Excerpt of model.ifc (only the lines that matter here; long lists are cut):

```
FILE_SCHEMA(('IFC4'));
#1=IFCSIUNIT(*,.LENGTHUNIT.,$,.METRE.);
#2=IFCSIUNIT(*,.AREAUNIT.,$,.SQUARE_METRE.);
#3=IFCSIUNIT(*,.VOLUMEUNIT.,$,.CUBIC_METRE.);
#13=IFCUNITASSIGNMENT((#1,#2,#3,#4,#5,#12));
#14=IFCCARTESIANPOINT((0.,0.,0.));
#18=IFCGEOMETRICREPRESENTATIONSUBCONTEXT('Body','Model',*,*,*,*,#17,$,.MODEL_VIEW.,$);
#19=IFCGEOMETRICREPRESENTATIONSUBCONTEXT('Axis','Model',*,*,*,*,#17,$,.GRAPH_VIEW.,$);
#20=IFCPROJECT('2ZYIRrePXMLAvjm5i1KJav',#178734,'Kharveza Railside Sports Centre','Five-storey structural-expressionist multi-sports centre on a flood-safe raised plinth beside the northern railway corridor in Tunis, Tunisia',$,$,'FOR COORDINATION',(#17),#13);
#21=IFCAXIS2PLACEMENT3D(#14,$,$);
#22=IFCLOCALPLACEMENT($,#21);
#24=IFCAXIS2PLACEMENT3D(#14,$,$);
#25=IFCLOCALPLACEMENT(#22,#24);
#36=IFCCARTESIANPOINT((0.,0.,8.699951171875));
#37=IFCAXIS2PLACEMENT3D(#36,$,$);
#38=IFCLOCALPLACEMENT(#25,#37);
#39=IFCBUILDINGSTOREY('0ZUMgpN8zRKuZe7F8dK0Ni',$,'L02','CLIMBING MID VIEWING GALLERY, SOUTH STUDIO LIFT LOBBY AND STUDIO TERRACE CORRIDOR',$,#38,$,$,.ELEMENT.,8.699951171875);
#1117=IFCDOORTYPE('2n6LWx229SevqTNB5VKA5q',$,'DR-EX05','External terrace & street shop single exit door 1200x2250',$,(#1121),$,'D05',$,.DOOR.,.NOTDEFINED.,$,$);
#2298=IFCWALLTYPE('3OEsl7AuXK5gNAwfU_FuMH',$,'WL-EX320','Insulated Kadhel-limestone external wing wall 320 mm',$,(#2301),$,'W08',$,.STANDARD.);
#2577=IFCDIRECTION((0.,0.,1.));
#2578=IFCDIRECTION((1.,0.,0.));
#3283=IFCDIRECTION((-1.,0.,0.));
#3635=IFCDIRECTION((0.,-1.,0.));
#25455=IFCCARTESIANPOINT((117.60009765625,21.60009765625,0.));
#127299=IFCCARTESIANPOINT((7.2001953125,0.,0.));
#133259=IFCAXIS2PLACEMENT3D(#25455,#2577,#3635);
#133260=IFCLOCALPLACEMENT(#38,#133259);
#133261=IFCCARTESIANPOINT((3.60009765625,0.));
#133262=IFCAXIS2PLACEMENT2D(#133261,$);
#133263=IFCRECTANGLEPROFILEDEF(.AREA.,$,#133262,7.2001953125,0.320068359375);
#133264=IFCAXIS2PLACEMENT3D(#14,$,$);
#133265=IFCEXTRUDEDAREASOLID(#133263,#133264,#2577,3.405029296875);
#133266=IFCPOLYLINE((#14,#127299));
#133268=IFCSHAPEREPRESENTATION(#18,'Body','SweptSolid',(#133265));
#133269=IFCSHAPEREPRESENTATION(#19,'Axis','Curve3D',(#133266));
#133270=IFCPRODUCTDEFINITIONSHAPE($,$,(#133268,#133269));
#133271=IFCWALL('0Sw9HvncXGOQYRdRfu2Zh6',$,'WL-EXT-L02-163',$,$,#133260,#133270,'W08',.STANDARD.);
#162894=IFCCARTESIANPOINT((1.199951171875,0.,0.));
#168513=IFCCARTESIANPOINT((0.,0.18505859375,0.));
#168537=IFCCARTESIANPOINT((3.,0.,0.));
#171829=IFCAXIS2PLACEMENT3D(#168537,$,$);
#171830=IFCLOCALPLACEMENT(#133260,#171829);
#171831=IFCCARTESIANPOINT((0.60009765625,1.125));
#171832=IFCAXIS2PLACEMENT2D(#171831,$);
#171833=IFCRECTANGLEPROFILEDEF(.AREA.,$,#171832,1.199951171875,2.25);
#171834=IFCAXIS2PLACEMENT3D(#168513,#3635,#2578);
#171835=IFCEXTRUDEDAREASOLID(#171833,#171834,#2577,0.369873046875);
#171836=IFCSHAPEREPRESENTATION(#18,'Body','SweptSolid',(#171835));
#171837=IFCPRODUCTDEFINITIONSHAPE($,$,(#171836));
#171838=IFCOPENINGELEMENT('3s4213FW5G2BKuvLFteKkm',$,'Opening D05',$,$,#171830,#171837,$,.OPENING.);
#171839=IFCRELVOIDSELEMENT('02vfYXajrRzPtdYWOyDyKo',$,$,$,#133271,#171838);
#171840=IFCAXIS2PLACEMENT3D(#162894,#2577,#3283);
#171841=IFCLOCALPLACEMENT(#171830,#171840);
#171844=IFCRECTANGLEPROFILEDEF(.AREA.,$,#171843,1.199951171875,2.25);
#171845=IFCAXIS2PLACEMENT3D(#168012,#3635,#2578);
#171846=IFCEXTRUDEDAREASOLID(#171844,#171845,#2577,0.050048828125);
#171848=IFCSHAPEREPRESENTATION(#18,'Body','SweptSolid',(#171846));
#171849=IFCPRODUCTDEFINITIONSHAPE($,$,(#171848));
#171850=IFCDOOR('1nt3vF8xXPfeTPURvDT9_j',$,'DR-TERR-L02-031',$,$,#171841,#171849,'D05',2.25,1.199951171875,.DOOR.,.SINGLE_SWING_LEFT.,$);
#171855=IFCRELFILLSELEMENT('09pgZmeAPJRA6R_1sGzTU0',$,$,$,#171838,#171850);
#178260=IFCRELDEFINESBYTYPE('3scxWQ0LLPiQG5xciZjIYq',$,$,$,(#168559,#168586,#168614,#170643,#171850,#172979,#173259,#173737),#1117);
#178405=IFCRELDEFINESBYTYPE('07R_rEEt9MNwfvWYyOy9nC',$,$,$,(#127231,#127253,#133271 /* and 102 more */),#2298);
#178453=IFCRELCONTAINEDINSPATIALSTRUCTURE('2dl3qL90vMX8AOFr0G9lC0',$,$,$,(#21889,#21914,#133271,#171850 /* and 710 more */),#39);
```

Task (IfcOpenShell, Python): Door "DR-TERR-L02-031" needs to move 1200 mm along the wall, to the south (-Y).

```python
import ifcopenshell
import ifcopenshell.api.geometry
import ifcopenshell.util.placement

model = ifcopenshell.open("model.ifc")

door = model.by_guid("1nt3vF8xXPfeTPURvDT9_j")
opening = door.FillsVoids[0].RelatingOpeningElement
wall = opening.VoidsElements[0].RelatingBuildingElement

wall_matrix = ifcopenshell.util.placement.get_local_placement(wall.ObjectPlacement)
shift = wall_matrix[:3, 0] * 1.2
before = ifcopenshell.util.placement.get_local_placement(door.ObjectPlacement)[:3, 3].copy()

# The door is placed relative to its opening, so it follows when the opening moves.
matrix = ifcopenshell.util.placement.get_local_placement(opening.ObjectPlacement)
matrix[:3, 3] += shift
ifcopenshell.api.geometry.edit_object_placement(
    model, product=opening, matrix=matrix, is_si=False, should_transform_children=True
)

after = ifcopenshell.util.placement.get_local_placement(door.ObjectPlacement)[:3, 3]
print("door moved by", (after - before).round(3) + 0.0)

model.write("model_updated.ifc")
```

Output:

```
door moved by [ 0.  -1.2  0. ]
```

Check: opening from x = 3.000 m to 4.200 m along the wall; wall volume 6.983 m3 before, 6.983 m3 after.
